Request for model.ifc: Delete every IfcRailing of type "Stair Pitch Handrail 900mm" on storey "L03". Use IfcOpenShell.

First a look at what the model holds.

```python
import ifcopenshell
import ifcopenshell.util.element

model = ifcopenshell.open("model.ifc")
print(model.schema)
storey = next(s for s in model.by_type("IfcBuildingStorey") if s.Name == "L03")
railings = [e for e in ifcopenshell.util.element.get_decomposition(storey) if e.is_a("IfcRailing")]
seen = {}
for e in railings:
    element_type = ifcopenshell.util.element.get_type(e)
    name = element_type.Name if element_type not in (None, e) else None
    seen[name] = seen.get(name, 0) + 1
for name, count in sorted(seen.items(), key=str):
    print(count, "x", name)
```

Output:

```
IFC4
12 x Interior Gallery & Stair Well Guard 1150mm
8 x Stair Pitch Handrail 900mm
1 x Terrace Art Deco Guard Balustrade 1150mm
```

```python
import ifcopenshell
import ifcopenshell.api.root
import ifcopenshell.util.element

model = ifcopenshell.open("model.ifc")

storey = next(s for s in model.by_type("IfcBuildingStorey") if s.Name == "L03")
railings = [e for e in ifcopenshell.util.element.get_decomposition(storey) if e.is_a("IfcRailing")]
targets = [e for e in railings if (t := ifcopenshell.util.element.get_type(e)) not in (None, e) and t.Name == "Stair Pitch Handrail 900mm"]

for e in targets:
    ifcopenshell.api.root.remove_product(model, product=e)
print(len(targets), "removed")

model.write("model-out.ifc")
```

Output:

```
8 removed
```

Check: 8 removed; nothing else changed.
